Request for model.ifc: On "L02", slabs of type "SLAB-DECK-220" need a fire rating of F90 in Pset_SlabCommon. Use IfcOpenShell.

First a look at what the model holds.

```python
import ifcopenshell
import ifcopenshell.util.element

model = ifcopenshell.open("model.ifc")
print(model.schema)
storey = next(s for s in model.by_type("IfcBuildingStorey") if s.Name == "L02")
slabs = [e for e in ifcopenshell.util.element.get_decomposition(storey) if e.is_a("IfcSlab")]
seen = {}
for e in slabs:
    element_type = ifcopenshell.util.element.get_type(e)
    key = (element_type.Name if element_type != e and element_type else None, ifcopenshell.util.element.get_pset(e, "Pset_SlabCommon", "FireRating"))
    seen[key] = seen.get(key, 0) + 1
for (name, value), count in sorted(seen.items(), key=str):
    print(count, "x", name, "|", value)
```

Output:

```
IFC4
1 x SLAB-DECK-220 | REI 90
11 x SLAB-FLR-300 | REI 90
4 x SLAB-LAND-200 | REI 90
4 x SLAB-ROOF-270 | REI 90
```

```python
import ifcopenshell
import ifcopenshell.api.pset
import ifcopenshell.util.element

model = ifcopenshell.open("model.ifc")

storey = next(s for s in model.by_type("IfcBuildingStorey") if s.Name == "L02")
slabs = [e for e in ifcopenshell.util.element.get_decomposition(storey) if e.is_a("IfcSlab")]

count = 0
for e in slabs:
    element_type = ifcopenshell.util.element.get_type(e)
    if element_type in (None, e) or element_type.Name != "SLAB-DECK-220":
        continue
    # add_pset returns the element's existing set when there is one.
    pset = ifcopenshell.api.pset.add_pset(model, product=e, name="Pset_SlabCommon")
    ifcopenshell.api.pset.edit_pset(model, pset=pset, properties={"FireRating": "F90"})
    count += 1

print(count, "slabs updated")

model.write("model_rev.ifc")
```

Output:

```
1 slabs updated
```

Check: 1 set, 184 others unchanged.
